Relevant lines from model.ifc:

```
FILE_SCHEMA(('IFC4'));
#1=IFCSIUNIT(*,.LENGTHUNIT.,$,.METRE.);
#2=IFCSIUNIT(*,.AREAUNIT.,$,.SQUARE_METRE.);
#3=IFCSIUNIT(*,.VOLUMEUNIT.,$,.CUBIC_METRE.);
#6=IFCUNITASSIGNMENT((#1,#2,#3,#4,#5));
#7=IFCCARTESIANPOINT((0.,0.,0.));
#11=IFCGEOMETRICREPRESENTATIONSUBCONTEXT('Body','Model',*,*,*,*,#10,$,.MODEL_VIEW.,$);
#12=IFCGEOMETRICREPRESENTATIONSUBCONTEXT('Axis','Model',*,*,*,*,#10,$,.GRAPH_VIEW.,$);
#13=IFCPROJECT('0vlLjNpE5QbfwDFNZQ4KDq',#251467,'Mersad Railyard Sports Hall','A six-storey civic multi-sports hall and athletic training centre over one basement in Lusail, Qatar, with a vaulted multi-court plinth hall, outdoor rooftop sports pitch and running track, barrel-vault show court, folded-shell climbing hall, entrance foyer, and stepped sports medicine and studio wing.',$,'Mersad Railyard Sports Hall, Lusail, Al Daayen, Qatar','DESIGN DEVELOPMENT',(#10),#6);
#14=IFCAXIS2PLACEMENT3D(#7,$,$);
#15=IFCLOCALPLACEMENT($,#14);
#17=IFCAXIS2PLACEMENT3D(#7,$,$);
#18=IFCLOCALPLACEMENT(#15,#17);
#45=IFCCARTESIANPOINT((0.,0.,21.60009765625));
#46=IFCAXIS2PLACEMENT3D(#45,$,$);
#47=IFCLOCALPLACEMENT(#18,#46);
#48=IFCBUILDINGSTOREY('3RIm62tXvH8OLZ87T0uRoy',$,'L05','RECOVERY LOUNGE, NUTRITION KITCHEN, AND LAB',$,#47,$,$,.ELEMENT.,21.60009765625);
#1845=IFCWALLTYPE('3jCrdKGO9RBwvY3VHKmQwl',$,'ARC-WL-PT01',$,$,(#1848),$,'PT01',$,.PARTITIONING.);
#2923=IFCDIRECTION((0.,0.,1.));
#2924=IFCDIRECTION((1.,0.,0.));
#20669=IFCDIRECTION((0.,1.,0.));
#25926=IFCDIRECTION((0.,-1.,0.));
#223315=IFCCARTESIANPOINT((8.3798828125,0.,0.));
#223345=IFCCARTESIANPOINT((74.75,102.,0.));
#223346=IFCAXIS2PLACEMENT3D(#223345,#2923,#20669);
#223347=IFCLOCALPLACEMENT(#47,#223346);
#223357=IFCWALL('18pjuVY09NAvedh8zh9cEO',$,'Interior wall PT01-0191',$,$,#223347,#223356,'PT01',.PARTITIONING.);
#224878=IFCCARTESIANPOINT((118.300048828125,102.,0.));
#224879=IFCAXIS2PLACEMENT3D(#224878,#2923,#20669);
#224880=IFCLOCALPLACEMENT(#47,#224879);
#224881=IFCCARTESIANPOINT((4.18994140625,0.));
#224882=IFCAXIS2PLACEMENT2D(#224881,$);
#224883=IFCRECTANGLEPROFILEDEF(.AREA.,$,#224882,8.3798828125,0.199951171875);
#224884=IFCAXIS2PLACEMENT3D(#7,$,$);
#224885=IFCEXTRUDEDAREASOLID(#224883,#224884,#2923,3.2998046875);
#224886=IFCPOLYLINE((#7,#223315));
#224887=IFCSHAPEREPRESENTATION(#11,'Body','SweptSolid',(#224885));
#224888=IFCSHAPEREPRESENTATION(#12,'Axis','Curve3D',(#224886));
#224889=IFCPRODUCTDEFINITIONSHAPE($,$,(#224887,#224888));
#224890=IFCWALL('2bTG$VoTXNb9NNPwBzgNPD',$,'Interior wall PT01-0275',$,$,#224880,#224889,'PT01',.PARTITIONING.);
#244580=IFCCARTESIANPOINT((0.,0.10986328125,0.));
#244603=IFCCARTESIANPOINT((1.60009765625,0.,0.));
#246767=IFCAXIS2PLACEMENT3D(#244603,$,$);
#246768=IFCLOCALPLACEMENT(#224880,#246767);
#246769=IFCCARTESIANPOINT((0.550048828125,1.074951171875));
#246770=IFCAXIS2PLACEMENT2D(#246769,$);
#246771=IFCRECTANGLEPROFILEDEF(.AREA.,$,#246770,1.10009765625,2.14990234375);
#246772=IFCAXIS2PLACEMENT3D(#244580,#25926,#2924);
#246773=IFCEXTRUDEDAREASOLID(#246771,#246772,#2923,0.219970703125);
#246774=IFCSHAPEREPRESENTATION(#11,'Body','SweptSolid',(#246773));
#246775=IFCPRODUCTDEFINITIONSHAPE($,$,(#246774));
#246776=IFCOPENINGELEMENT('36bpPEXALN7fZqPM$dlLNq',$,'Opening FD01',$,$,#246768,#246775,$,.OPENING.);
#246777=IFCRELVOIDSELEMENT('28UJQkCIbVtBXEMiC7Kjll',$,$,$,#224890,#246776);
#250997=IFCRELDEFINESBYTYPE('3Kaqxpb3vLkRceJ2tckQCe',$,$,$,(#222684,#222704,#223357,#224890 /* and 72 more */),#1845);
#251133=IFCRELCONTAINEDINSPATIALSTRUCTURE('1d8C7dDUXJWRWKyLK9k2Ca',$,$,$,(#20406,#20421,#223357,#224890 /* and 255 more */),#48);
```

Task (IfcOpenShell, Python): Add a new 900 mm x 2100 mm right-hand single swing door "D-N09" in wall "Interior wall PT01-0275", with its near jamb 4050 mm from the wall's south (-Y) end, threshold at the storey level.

```python
import numpy as np
import ifcopenshell
import ifcopenshell.api.feature
import ifcopenshell.api.geometry
import ifcopenshell.api.root
import ifcopenshell.api.spatial
import ifcopenshell.geom
import ifcopenshell.util.element
import ifcopenshell.util.placement
import ifcopenshell.util.representation
import ifcopenshell.util.shape
import ifcopenshell.util.unit

model = ifcopenshell.open("model.ifc")
unit_scale = ifcopenshell.util.unit.calculate_unit_scale(model)
settings = ifcopenshell.geom.settings()


def volume(element):
    """Net volume in cubic metres, openings subtracted."""
    shape = ifcopenshell.geom.create_shape(settings, element)
    return ifcopenshell.util.shape.get_volume(shape.geometry)


wall = model.by_guid("2bTG$VoTXNb9NNPwBzgNPD")
storey = ifcopenshell.util.element.get_container(wall, ifc_class="IfcBuildingStorey")
context = ifcopenshell.util.representation.get_context(model, "Model", "Body", "MODEL_VIEW")
before = volume(wall)

width, height, from_end, sill = 0.9, 2.1, 4.05, 0.0  # metres

# The wall runs along its own X axis, and the end named is its -X end.
wall_shape = ifcopenshell.geom.create_shape(settings, wall)
x, y, z = ifcopenshell.util.shape.get_vertices(wall_shape.geometry).T
start = x.min() + from_end
face, thickness = float(y.min()), float(y.max() - y.min())
wall_matrix = ifcopenshell.util.placement.get_local_placement(wall.ObjectPlacement)
level = ifcopenshell.util.placement.get_local_placement(storey.ObjectPlacement)[2, 3]


def in_wall(x, y):
    """Placement at x, y metres in the wall's axes, at sill height."""
    matrix = wall_matrix.copy()
    matrix[:, 3] = wall_matrix @ np.array([x / unit_scale, y / unit_scale, 0.0, 1.0])
    matrix[2, 3] = level + sill / unit_scale
    return matrix


# Opening: a box that overshoots both wall faces by 50 mm.
opening = ifcopenshell.api.root.create_entity(model, ifc_class="IfcOpeningElement", predefined_type="OPENING")
box = ifcopenshell.api.geometry.add_wall_representation(
    model, context=context, length=width, height=height, thickness=thickness + 0.1
)
ifcopenshell.api.geometry.assign_representation(model, product=opening, representation=box)
ifcopenshell.api.geometry.edit_object_placement(model, product=opening, matrix=in_wall(start, face - 0.05), is_si=False)
ifcopenshell.api.feature.add_feature(model, feature=opening, element=wall)

door = ifcopenshell.api.root.create_entity(model, ifc_class="IfcDoor", name="D-N09", predefined_type="DOOR")
door.OverallWidth, door.OverallHeight = width / unit_scale, height / unit_scale
door.OperationType = "SINGLE_SWING_RIGHT"
body = ifcopenshell.api.geometry.add_door_representation(
    model,
    context=context,
    overall_width=door.OverallWidth,
    overall_height=door.OverallHeight,
    operation_type="SINGLE_SWING_RIGHT",
    lining_properties={"LiningDepth": thickness / unit_scale, "ThresholdDepth": thickness / unit_scale},
)
ifcopenshell.api.geometry.assign_representation(model, product=door, representation=body)
ifcopenshell.api.spatial.assign_container(model, products=[door], relating_structure=storey)
ifcopenshell.api.feature.add_filling(model, opening=opening, element=door)

# The lining spans the wall, so the door starts at the wall face.
ifcopenshell.api.geometry.edit_object_placement(model, product=door, matrix=in_wall(start, face), is_si=False)

after = volume(wall)

print(f"wall volume {before:.3f} -> {after:.3f} m3")

model.write("model_edited.ifc")
```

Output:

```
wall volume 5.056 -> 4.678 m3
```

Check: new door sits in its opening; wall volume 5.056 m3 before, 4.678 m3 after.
